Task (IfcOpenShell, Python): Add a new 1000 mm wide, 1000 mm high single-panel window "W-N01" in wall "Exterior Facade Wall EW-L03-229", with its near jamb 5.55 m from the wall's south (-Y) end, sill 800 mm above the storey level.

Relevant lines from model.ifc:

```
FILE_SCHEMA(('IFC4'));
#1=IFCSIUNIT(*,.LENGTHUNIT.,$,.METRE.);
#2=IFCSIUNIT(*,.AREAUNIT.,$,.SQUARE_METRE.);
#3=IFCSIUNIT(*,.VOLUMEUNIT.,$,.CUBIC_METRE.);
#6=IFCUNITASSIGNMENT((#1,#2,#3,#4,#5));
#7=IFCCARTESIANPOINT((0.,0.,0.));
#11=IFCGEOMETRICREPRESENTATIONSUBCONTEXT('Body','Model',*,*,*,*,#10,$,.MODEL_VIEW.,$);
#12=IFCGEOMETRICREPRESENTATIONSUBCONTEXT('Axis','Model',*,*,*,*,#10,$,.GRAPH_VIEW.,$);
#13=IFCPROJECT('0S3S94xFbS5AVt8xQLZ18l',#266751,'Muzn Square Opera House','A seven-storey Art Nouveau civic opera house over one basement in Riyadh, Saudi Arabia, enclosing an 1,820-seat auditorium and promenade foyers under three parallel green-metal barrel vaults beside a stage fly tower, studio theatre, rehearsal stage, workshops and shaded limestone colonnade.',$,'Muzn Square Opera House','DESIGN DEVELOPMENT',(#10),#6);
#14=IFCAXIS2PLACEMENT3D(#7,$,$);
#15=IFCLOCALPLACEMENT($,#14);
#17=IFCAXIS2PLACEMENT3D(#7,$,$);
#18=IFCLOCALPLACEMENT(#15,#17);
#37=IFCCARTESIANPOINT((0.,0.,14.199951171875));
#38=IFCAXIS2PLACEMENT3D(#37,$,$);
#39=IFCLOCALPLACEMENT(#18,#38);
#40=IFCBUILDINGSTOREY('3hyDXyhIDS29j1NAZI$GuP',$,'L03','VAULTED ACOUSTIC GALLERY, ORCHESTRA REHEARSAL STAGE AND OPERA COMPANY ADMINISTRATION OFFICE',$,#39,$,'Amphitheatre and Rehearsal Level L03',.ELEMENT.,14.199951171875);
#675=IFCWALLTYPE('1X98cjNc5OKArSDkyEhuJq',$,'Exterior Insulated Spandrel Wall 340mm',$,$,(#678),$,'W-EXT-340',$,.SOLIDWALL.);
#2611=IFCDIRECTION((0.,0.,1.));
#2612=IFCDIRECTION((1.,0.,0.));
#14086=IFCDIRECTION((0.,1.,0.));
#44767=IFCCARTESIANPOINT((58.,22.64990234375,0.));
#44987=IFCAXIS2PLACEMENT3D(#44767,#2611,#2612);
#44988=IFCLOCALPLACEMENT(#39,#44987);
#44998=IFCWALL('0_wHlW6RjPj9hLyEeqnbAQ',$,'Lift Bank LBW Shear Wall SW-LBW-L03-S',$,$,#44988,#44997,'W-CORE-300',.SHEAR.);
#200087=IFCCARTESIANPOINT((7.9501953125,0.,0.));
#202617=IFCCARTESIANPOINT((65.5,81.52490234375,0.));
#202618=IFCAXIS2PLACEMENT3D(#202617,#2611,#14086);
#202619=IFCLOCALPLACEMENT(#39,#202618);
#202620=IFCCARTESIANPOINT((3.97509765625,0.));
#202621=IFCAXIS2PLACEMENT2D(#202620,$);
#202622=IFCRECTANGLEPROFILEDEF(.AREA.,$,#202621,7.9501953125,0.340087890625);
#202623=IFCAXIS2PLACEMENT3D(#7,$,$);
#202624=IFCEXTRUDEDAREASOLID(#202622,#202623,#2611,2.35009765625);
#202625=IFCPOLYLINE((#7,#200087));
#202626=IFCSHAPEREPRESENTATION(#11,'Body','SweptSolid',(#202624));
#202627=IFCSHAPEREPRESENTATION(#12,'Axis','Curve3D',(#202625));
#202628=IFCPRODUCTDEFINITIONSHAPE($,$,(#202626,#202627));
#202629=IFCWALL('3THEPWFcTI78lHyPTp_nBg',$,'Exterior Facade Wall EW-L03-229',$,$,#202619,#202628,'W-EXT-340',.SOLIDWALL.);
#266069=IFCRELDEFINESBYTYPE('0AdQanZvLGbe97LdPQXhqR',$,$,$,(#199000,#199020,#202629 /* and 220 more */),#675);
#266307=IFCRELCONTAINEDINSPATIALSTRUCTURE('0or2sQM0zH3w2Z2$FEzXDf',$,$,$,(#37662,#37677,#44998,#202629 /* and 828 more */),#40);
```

```python
import numpy as np
import ifcopenshell
import ifcopenshell.api.feature
import ifcopenshell.api.geometry
import ifcopenshell.api.root
import ifcopenshell.api.spatial
import ifcopenshell.geom
import ifcopenshell.util.element
import ifcopenshell.util.placement
import ifcopenshell.util.representation
import ifcopenshell.util.shape
import ifcopenshell.util.unit

model = ifcopenshell.open("model.ifc")
unit_scale = ifcopenshell.util.unit.calculate_unit_scale(model)
settings = ifcopenshell.geom.settings()


def volume(element):
    """Net volume in cubic metres, openings subtracted."""
    shape = ifcopenshell.geom.create_shape(settings, element)
    return ifcopenshell.util.shape.get_volume(shape.geometry)


wall = model.by_guid("3THEPWFcTI78lHyPTp_nBg")
storey = ifcopenshell.util.element.get_container(wall, ifc_class="IfcBuildingStorey")
context = ifcopenshell.util.representation.get_context(model, "Model", "Body", "MODEL_VIEW")
before = volume(wall)

width, height, from_end, sill = 1, 1, 5.55, 0.8  # metres

# The wall runs along its own X axis, and the end named is its -X end.
wall_shape = ifcopenshell.geom.create_shape(settings, wall)
x, y, z = ifcopenshell.util.shape.get_vertices(wall_shape.geometry).T
start = x.min() + from_end
face, thickness = float(y.min()), float(y.max() - y.min())
wall_matrix = ifcopenshell.util.placement.get_local_placement(wall.ObjectPlacement)
level = ifcopenshell.util.placement.get_local_placement(storey.ObjectPlacement)[2, 3]


def in_wall(x, y):
    """Placement at x, y metres in the wall's axes, at sill height."""
    matrix = wall_matrix.copy()
    matrix[:, 3] = wall_matrix @ np.array([x / unit_scale, y / unit_scale, 0.0, 1.0])
    matrix[2, 3] = level + sill / unit_scale
    return matrix


# Opening: a box that overshoots both wall faces by 50 mm.
opening = ifcopenshell.api.root.create_entity(model, ifc_class="IfcOpeningElement", predefined_type="OPENING")
box = ifcopenshell.api.geometry.add_wall_representation(
    model, context=context, length=width, height=height, thickness=thickness + 0.1
)
ifcopenshell.api.geometry.assign_representation(model, product=opening, representation=box)
ifcopenshell.api.geometry.edit_object_placement(model, product=opening, matrix=in_wall(start, face - 0.05), is_si=False)
ifcopenshell.api.feature.add_feature(model, feature=opening, element=wall)

window = ifcopenshell.api.root.create_entity(model, ifc_class="IfcWindow", name="W-N01", predefined_type="WINDOW")
window.OverallWidth, window.OverallHeight = width / unit_scale, height / unit_scale
window.PartitioningType = "SINGLE_PANEL"
body = ifcopenshell.api.geometry.add_window_representation(
    model,
    context=context,
    overall_width=window.OverallWidth,
    overall_height=window.OverallHeight,
    partition_type="SINGLE_PANEL",
)
ifcopenshell.api.geometry.assign_representation(model, product=window, representation=body)
ifcopenshell.api.spatial.assign_container(model, products=[window], relating_structure=storey)
ifcopenshell.api.feature.add_filling(model, opening=opening, element=window)

# Centre the window in the wall's thickness.
ifcopenshell.api.geometry.edit_object_placement(model, product=window, matrix=in_wall(start, face), is_si=False)
window_shape = ifcopenshell.geom.create_shape(settings, window)
depth = ifcopenshell.util.shape.get_vertices(window_shape.geometry)[:, 1]
offset = face + thickness / 2 - (depth.min() + depth.max()) / 2
ifcopenshell.api.geometry.edit_object_placement(model, product=window, matrix=in_wall(start, offset), is_si=False)

after = volume(wall)

print(f"wall volume {before:.3f} -> {after:.3f} m3")

model.write("model_edited.ifc")
```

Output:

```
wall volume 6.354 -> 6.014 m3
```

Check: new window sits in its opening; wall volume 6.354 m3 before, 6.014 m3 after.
